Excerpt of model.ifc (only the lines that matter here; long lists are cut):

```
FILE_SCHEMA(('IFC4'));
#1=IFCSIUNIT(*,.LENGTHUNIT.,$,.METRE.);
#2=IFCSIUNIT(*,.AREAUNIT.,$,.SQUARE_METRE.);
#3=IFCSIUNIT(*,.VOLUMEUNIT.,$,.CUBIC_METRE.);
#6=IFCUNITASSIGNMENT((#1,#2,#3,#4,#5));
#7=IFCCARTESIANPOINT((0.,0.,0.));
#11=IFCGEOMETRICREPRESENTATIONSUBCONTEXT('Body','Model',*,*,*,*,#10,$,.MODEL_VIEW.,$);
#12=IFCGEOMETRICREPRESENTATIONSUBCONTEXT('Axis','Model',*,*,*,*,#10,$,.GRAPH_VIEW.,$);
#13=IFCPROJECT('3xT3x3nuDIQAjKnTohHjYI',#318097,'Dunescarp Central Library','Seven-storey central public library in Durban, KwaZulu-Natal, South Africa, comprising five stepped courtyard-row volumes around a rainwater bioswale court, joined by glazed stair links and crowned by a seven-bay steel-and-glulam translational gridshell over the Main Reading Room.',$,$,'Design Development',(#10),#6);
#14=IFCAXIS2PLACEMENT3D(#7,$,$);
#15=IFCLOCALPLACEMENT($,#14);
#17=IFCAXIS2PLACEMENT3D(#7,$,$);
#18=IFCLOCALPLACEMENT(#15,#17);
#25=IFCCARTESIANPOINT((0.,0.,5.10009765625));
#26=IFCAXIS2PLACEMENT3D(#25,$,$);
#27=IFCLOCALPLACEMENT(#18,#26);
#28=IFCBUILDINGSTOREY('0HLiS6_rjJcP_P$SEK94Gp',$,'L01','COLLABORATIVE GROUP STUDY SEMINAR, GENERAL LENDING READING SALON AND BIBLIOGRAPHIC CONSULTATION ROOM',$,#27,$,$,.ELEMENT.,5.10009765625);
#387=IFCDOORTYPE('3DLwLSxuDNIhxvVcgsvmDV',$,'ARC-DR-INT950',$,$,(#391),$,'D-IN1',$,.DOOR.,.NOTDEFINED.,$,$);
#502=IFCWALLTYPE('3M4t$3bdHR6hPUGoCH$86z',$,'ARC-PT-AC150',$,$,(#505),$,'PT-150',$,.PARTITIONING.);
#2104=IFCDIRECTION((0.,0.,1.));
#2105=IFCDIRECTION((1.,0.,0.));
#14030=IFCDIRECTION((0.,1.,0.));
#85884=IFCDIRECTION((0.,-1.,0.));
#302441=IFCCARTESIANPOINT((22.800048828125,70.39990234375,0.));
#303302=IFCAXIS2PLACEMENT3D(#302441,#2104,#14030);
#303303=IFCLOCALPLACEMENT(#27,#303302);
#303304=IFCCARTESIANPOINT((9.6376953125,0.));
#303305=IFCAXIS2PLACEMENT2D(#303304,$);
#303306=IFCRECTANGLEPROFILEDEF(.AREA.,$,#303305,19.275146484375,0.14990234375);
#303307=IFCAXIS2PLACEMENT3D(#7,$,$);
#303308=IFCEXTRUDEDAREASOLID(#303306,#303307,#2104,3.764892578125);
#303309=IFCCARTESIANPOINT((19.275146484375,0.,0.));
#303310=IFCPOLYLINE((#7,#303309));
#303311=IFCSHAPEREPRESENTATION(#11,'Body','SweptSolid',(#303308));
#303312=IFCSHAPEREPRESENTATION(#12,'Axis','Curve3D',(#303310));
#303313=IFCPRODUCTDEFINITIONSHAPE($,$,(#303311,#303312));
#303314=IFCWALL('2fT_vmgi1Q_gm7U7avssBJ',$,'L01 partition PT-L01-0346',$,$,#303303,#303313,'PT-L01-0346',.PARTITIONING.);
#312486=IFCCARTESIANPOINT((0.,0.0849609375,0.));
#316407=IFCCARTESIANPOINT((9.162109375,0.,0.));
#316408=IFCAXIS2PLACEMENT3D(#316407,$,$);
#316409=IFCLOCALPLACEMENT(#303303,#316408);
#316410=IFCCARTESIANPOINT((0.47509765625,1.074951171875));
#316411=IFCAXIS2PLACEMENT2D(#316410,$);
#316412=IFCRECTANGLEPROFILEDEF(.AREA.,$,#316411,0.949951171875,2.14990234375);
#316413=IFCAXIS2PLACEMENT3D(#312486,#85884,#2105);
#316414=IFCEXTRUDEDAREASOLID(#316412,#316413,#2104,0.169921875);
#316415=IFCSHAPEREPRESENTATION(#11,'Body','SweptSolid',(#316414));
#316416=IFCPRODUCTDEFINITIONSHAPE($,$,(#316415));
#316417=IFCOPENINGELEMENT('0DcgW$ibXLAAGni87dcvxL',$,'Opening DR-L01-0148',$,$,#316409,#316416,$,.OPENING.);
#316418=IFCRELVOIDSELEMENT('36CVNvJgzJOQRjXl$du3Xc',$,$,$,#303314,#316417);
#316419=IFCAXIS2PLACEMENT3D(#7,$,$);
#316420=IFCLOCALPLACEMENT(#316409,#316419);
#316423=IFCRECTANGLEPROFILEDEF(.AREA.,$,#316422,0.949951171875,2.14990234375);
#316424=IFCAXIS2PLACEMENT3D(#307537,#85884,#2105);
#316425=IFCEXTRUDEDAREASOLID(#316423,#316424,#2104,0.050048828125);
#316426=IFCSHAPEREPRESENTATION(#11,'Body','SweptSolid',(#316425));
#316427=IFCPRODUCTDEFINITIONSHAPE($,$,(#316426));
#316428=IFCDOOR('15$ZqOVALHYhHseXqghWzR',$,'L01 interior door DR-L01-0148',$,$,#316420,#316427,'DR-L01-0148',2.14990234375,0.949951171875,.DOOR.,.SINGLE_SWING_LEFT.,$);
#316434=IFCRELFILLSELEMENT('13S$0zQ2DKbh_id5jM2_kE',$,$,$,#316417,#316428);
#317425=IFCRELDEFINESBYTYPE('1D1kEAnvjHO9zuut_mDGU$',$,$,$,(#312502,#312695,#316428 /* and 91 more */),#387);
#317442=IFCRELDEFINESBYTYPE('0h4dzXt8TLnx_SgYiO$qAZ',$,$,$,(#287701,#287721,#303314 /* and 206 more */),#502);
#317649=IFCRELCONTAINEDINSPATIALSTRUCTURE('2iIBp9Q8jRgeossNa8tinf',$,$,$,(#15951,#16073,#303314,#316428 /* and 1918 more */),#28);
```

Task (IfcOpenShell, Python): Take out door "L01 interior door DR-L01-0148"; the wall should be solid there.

```python
import ifcopenshell
import ifcopenshell.api.feature
import ifcopenshell.api.root
import ifcopenshell.geom
import ifcopenshell.util.shape

model = ifcopenshell.open("model.ifc")
settings = ifcopenshell.geom.settings()


def volume(element):
    """Net volume in cubic metres, openings subtracted."""
    shape = ifcopenshell.geom.create_shape(settings, element)
    return ifcopenshell.util.shape.get_volume(shape.geometry)


door = model.by_guid("15$ZqOVALHYhHseXqghWzR")
opening = door.FillsVoids[0].RelatingOpeningElement
wall = opening.VoidsElements[0].RelatingBuildingElement
before = volume(wall)

ifcopenshell.api.root.remove_product(model, product=door)
ifcopenshell.api.feature.remove_feature(model, feature=opening)

after = volume(wall)

print(f"wall volume {before:.3f} -> {after:.3f} m3")

model.write("model_v2.ifc")
```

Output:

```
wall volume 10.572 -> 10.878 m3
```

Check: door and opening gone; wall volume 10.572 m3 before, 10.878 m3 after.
